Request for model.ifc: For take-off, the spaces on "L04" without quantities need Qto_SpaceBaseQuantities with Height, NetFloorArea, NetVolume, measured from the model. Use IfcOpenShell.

First a look at what the model holds.

```python
import ifcopenshell
import ifcopenshell.util.element
import ifcopenshell.util.unit

model = ifcopenshell.open("model.ifc")
print(model.schema)
for unit_type in ("LENGTHUNIT", "AREAUNIT", "VOLUMEUNIT"):
    print(unit_type, ifcopenshell.util.unit.calculate_unit_scale(model, unit_type))
storey = next(s for s in model.by_type("IfcBuildingStorey") if s.Name == "L04")
spaces = [e for e in ifcopenshell.util.element.get_decomposition(storey) if e.is_a("IfcSpace")]
for e in sorted(spaces, key=lambda e: e.id()):
    print(e.id(), e.is_a(), e.Name, list(ifcopenshell.util.element.get_psets(e, qtos_only=True)), sep=" | ")
```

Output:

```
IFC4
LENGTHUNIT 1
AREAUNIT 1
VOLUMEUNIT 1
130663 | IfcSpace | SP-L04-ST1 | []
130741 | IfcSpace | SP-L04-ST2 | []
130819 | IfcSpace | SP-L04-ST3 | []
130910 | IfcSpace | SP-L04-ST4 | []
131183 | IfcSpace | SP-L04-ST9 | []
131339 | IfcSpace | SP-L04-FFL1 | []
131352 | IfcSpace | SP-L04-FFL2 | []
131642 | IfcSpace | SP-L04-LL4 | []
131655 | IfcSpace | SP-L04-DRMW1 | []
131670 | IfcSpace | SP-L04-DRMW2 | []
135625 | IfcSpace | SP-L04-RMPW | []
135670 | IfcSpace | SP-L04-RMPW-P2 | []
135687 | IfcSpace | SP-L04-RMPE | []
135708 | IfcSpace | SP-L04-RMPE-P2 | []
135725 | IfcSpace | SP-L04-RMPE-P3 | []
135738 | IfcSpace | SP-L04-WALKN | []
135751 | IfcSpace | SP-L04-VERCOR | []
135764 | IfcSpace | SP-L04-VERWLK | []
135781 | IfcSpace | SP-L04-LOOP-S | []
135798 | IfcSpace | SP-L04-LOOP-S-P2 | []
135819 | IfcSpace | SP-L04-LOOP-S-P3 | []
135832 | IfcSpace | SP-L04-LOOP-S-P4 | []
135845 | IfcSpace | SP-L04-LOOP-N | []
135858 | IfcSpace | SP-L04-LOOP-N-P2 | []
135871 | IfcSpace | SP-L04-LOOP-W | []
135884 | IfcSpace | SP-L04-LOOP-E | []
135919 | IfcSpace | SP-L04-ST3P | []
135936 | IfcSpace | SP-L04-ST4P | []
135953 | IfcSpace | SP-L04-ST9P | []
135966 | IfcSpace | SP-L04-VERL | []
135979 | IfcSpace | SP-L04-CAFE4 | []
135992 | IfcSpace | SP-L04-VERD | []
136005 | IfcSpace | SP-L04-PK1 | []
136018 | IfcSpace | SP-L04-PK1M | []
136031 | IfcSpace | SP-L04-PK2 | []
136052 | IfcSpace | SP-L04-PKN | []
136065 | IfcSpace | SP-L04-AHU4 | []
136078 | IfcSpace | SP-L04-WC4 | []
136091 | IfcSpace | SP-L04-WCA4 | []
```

```python
import ifcopenshell
import ifcopenshell.api.pset
import ifcopenshell.geom
import ifcopenshell.util.element
import ifcopenshell.util.shape
import ifcopenshell.util.unit

model = ifcopenshell.open("model.ifc")
unit_scale = ifcopenshell.util.unit.calculate_unit_scale(model)
area_scale = ifcopenshell.util.unit.calculate_unit_scale(model, "AREAUNIT")
volume_scale = ifcopenshell.util.unit.calculate_unit_scale(model, "VOLUMEUNIT")
settings = ifcopenshell.geom.settings()

storey = next(s for s in model.by_type("IfcBuildingStorey") if s.Name == "L04")
spaces = [e for e in ifcopenshell.util.element.get_decomposition(storey) if e.is_a("IfcSpace")]

for e in sorted(spaces, key=lambda e: e.id()):
    if ifcopenshell.util.element.get_psets(e, qtos_only=True, should_inherit=False):
        continue
    # Geometry comes back in metres, in the element's own axes.
    shape = ifcopenshell.geom.create_shape(settings, e)
    values = {
        "Height": ifcopenshell.util.shape.get_z(shape.geometry) / unit_scale,
        "NetFloorArea": ifcopenshell.util.shape.get_footprint_area(shape.geometry) / area_scale,
        "NetVolume": ifcopenshell.util.shape.get_volume(shape.geometry) / volume_scale,
    }
    qto = ifcopenshell.api.pset.add_qto(model, product=e, name="Qto_SpaceBaseQuantities")
    ifcopenshell.api.pset.edit_qto(model, qto=qto, properties=values)
    print(e.id(), {k: round(v, 3) for k, v in values.items()})

model.write("model_updated.ifc")
```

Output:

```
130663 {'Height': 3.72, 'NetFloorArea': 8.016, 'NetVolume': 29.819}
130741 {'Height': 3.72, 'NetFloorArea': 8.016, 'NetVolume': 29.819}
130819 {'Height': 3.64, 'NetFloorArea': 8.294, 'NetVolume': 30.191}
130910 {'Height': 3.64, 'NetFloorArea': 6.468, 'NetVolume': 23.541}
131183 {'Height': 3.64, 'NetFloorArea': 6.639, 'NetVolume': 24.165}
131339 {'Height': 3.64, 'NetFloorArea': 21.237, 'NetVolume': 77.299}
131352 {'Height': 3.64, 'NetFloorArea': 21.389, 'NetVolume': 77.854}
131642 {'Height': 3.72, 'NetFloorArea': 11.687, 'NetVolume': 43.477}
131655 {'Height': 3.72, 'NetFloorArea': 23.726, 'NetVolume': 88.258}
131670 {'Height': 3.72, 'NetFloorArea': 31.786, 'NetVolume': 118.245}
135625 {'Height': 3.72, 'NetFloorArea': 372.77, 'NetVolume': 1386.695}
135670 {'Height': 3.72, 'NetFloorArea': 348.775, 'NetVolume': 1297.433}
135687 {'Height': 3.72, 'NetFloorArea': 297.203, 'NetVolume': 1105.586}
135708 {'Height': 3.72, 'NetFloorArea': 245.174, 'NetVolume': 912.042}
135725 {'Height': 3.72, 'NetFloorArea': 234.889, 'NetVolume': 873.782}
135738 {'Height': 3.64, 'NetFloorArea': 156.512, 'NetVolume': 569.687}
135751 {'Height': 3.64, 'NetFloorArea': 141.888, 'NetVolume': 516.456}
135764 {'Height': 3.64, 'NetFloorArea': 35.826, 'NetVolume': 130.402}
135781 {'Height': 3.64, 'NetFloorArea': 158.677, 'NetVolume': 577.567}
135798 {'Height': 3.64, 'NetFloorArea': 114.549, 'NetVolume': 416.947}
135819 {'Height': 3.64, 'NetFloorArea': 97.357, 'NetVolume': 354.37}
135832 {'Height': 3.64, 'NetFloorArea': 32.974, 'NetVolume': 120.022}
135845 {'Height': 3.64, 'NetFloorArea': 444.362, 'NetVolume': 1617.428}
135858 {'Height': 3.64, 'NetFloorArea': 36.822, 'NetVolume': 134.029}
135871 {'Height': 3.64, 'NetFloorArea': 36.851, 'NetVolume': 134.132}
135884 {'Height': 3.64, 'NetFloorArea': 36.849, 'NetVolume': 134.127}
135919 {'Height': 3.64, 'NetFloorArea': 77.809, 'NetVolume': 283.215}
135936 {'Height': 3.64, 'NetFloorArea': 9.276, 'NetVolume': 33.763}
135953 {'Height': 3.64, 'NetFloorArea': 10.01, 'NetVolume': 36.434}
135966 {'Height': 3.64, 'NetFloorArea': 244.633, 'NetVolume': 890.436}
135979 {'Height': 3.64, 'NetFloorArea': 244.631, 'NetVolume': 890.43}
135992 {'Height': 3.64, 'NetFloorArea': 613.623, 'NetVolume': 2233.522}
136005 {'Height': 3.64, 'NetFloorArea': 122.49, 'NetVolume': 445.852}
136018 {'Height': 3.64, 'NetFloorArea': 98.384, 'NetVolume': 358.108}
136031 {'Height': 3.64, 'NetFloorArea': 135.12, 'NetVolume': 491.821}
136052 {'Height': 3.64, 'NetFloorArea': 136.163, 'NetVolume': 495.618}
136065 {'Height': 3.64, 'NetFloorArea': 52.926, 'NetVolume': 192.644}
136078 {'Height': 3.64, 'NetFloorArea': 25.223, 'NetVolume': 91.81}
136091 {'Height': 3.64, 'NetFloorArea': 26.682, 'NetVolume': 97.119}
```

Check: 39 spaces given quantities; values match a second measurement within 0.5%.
